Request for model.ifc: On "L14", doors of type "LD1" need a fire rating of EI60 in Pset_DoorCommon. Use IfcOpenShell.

First a look at what the model holds.

```python
import ifcopenshell
import ifcopenshell.util.element

model = ifcopenshell.open("model.ifc")
print(model.schema)
storey = next(s for s in model.by_type("IfcBuildingStorey") if s.Name == "L14")
doors = [e for e in ifcopenshell.util.element.get_decomposition(storey) if e.is_a("IfcDoor")]
seen = {}
for e in doors:
    element_type = ifcopenshell.util.element.get_type(e)
    key = (element_type.Name if element_type != e and element_type else None, ifcopenshell.util.element.get_pset(e, "Pset_DoorCommon", "FireRating"))
    seen[key] = seen.get(key, 0) + 1
for (name, value), count in sorted(seen.items(), key=str):
    print(count, "x", name, "|", value)
```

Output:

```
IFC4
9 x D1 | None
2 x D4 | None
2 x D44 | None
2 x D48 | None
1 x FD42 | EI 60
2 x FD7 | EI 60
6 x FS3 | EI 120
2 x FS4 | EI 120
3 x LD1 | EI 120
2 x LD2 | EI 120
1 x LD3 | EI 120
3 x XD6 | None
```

```python
import ifcopenshell
import ifcopenshell.api.pset
import ifcopenshell.util.element

model = ifcopenshell.open("model.ifc")

storey = next(s for s in model.by_type("IfcBuildingStorey") if s.Name == "L14")
doors = [e for e in ifcopenshell.util.element.get_decomposition(storey) if e.is_a("IfcDoor")]

count = 0
for e in doors:
    element_type = ifcopenshell.util.element.get_type(e)
    if element_type in (None, e) or element_type.Name != "LD1":
        continue
    # add_pset returns the element's existing set when there is one.
    pset = ifcopenshell.api.pset.add_pset(model, product=e, name="Pset_DoorCommon")
    ifcopenshell.api.pset.edit_pset(model, pset=pset, properties={"FireRating": "EI60"})
    count += 1

print(count, "doors updated")

model.write("model_rev.ifc")
```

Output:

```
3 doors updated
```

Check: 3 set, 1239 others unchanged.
